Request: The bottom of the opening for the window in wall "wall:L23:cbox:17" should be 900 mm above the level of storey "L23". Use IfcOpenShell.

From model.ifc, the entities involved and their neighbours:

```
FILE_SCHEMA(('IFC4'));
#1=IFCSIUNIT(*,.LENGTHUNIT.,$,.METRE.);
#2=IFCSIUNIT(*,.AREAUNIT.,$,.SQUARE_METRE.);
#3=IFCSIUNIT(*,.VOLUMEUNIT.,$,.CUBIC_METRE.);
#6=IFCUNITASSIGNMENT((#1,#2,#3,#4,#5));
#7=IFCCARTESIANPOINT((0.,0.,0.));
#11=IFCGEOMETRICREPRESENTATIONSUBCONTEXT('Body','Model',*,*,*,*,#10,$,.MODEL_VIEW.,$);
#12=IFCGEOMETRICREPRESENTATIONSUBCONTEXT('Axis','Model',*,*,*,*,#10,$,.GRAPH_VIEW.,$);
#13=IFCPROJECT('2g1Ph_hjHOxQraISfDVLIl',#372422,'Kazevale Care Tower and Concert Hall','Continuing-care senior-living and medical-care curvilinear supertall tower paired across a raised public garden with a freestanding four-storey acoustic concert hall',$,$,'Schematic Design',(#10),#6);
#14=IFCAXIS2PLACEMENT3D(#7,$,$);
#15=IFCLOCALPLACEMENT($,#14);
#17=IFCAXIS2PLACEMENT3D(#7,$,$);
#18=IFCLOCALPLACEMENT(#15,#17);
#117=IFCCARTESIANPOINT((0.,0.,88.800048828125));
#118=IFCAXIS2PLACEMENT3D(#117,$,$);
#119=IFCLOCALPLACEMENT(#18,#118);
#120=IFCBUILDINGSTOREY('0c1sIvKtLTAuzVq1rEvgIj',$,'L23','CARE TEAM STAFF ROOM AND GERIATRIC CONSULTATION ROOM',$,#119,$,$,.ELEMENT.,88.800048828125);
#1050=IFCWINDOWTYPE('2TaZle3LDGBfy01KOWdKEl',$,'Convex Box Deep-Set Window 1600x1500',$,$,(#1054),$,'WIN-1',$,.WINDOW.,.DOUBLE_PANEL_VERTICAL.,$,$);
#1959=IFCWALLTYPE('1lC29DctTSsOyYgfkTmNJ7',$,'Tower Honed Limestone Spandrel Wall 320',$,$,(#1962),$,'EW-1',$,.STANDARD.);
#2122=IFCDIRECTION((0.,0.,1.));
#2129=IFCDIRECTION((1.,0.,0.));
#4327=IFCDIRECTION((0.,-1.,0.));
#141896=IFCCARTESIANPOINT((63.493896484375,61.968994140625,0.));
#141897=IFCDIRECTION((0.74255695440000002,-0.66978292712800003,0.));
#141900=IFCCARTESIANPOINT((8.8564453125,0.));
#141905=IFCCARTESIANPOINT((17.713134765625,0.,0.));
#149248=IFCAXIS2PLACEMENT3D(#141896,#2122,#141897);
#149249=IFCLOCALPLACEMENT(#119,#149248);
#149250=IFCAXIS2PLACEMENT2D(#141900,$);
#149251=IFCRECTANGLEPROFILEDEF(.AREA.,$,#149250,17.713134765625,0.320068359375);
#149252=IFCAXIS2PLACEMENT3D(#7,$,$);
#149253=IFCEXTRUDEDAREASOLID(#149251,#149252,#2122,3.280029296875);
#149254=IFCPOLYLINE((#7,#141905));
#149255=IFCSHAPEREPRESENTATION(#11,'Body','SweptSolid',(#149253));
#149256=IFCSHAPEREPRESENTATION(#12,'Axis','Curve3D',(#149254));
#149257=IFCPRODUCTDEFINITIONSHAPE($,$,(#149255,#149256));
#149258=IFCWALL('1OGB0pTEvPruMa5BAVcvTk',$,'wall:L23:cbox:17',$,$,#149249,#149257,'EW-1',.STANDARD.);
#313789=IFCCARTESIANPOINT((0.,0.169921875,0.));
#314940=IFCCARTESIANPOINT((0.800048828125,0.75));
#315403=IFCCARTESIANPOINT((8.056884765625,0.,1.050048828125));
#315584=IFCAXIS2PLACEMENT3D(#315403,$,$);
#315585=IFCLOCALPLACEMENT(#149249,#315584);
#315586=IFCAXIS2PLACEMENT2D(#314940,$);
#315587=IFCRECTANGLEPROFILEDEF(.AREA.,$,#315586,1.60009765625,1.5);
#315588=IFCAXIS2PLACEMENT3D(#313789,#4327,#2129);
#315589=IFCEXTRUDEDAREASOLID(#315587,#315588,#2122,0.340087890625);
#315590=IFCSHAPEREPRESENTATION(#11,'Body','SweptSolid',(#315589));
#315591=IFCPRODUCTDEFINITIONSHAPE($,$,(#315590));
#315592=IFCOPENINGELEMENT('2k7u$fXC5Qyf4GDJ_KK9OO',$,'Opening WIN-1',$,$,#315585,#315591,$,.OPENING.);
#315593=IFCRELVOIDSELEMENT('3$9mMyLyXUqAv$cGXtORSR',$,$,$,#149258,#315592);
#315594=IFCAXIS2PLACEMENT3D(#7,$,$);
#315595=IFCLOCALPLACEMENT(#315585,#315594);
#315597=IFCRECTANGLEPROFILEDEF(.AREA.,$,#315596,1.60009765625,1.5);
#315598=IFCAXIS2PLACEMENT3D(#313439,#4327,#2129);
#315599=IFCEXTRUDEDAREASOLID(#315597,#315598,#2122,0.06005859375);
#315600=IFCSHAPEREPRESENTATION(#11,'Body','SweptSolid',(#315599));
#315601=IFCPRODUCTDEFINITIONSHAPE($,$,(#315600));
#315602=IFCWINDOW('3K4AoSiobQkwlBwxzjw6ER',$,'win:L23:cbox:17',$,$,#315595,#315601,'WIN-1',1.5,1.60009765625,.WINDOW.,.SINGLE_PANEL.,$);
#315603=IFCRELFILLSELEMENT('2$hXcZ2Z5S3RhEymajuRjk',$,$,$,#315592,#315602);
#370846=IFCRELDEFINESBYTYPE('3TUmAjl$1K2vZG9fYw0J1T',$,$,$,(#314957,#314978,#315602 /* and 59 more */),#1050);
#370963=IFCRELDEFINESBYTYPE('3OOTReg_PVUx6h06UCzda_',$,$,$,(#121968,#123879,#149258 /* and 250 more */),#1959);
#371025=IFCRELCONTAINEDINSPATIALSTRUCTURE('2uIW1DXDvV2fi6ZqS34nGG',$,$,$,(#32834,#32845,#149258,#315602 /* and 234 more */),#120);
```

```python
import numpy as np
import ifcopenshell
import ifcopenshell.api.geometry
import ifcopenshell.geom
import ifcopenshell.util.element
import ifcopenshell.util.placement
import ifcopenshell.util.shape
import ifcopenshell.util.unit

model = ifcopenshell.open("model.ifc")
unit_scale = ifcopenshell.util.unit.calculate_unit_scale(model)

window = model.by_id(315602)
opening = window.FillsVoids[0].RelatingOpeningElement
storey = ifcopenshell.util.element.get_container(window, ifc_class="IfcBuildingStorey")
level = ifcopenshell.util.placement.get_local_placement(storey.ObjectPlacement)[2, 3]

# The opening's origin need not be at the sill, so measure its lowest point.
shape = ifcopenshell.geom.create_shape(ifcopenshell.geom.settings(), opening)
bottom = ifcopenshell.util.shape.get_shape_bottom_elevation(shape, shape.geometry) / unit_scale
dz = level + 0.9 / unit_scale - bottom

shift = np.array([0.0, 0.0, dz])
# The window is placed relative to its opening, so it follows when the opening moves.
matrix = ifcopenshell.util.placement.get_local_placement(opening.ObjectPlacement)
matrix[:3, 3] += shift
ifcopenshell.api.geometry.edit_object_placement(
    model, product=opening, matrix=matrix, is_si=False, should_transform_children=True
)

print(f"moved by {dz * unit_scale:+.3f} m")

model.write("model_v2.ifc")
```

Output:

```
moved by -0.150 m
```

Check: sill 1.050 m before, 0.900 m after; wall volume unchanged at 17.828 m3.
